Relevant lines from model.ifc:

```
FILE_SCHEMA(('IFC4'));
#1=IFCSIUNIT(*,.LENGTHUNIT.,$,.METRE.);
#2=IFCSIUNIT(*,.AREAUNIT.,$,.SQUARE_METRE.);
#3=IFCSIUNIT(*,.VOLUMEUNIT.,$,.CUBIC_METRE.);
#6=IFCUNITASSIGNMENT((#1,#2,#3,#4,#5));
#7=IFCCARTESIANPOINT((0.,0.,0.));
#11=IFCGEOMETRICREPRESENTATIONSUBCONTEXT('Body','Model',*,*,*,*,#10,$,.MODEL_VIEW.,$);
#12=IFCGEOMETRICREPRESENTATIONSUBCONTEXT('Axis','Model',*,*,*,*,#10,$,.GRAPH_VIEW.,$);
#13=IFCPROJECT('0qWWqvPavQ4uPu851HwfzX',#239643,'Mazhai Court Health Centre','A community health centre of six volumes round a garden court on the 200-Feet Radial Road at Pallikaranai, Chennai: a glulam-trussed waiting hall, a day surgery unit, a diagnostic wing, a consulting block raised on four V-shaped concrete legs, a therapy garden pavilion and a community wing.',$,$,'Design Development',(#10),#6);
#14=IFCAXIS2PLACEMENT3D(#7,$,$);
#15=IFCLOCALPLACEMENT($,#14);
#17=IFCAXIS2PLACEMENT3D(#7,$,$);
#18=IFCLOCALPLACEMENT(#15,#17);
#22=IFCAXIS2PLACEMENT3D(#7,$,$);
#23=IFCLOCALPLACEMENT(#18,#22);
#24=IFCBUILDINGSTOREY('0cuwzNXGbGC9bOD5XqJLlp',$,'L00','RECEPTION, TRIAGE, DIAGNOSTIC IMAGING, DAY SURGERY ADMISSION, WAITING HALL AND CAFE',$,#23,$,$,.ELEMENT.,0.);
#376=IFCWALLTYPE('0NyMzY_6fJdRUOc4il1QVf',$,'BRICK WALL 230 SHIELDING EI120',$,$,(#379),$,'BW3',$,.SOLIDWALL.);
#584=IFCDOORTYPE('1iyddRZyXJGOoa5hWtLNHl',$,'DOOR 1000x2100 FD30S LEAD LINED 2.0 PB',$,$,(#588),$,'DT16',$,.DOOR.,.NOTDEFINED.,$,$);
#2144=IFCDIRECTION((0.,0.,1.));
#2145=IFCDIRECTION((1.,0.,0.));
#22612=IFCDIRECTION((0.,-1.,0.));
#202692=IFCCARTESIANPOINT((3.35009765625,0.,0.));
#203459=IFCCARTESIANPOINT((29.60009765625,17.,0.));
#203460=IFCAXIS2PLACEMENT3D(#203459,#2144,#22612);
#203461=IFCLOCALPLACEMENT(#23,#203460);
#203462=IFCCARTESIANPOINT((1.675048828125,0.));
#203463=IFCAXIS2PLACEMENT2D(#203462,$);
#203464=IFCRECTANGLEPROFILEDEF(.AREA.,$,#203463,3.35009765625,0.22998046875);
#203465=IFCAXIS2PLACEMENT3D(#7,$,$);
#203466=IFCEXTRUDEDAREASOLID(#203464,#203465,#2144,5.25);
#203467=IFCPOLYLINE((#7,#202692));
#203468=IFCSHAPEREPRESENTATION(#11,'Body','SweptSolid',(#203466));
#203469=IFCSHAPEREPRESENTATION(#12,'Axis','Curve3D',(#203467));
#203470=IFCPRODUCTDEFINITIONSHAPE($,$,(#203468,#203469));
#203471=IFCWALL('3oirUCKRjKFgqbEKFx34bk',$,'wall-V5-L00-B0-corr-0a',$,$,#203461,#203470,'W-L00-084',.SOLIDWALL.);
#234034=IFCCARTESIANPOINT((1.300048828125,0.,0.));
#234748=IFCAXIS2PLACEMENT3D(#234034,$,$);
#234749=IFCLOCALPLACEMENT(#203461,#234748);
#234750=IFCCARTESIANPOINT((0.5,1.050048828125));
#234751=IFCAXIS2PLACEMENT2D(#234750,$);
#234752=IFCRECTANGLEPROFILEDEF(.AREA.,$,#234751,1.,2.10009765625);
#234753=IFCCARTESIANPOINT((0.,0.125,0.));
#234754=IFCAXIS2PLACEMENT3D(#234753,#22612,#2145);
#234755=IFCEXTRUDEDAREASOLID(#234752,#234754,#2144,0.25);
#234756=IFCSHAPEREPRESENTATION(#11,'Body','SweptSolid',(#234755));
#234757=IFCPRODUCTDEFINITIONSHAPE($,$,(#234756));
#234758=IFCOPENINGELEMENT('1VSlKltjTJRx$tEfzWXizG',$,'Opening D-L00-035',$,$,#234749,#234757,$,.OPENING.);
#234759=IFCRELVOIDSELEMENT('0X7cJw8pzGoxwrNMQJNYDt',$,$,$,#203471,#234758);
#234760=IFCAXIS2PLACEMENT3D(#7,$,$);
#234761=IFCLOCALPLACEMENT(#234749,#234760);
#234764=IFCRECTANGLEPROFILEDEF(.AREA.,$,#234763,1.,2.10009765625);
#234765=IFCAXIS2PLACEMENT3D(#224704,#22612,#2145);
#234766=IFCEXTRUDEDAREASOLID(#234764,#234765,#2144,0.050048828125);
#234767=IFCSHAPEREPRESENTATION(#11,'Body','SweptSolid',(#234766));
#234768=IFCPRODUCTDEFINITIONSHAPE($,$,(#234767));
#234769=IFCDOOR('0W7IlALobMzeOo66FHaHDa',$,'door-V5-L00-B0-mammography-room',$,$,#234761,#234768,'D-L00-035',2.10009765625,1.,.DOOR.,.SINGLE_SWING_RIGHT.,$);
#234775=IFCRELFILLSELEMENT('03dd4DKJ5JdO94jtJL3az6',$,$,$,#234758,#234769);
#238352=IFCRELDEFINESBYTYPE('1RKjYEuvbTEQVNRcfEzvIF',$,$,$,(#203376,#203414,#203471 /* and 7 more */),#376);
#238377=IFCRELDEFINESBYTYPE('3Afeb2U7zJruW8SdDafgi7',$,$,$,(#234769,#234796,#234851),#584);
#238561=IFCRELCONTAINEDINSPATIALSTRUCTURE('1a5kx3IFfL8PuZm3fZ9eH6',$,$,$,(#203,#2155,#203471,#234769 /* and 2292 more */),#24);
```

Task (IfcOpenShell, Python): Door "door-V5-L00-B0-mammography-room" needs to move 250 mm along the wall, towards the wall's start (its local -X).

```python
import ifcopenshell
import ifcopenshell.api.geometry
import ifcopenshell.util.placement
import ifcopenshell.util.unit

model = ifcopenshell.open("model.ifc")
unit_scale = ifcopenshell.util.unit.calculate_unit_scale(model)

door = model.by_guid("0W7IlALobMzeOo66FHaHDa")
opening = door.FillsVoids[0].RelatingOpeningElement
wall = opening.VoidsElements[0].RelatingBuildingElement

wall_matrix = ifcopenshell.util.placement.get_local_placement(wall.ObjectPlacement)
shift = wall_matrix[:3, 0] * -0.25 / unit_scale
before = ifcopenshell.util.placement.get_local_placement(door.ObjectPlacement)[:3, 3].copy()

# The door is placed relative to its opening, so it follows when the opening moves.
matrix = ifcopenshell.util.placement.get_local_placement(opening.ObjectPlacement)
matrix[:3, 3] += shift
ifcopenshell.api.geometry.edit_object_placement(
    model, product=opening, matrix=matrix, is_si=False, should_transform_children=True
)

after = ifcopenshell.util.placement.get_local_placement(door.ObjectPlacement)[:3, 3]
print("door moved by", (after - before).round(3) + 0.0)

model.write("model_v2.ifc")
```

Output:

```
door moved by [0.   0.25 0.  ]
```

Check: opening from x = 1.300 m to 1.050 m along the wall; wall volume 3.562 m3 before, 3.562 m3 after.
